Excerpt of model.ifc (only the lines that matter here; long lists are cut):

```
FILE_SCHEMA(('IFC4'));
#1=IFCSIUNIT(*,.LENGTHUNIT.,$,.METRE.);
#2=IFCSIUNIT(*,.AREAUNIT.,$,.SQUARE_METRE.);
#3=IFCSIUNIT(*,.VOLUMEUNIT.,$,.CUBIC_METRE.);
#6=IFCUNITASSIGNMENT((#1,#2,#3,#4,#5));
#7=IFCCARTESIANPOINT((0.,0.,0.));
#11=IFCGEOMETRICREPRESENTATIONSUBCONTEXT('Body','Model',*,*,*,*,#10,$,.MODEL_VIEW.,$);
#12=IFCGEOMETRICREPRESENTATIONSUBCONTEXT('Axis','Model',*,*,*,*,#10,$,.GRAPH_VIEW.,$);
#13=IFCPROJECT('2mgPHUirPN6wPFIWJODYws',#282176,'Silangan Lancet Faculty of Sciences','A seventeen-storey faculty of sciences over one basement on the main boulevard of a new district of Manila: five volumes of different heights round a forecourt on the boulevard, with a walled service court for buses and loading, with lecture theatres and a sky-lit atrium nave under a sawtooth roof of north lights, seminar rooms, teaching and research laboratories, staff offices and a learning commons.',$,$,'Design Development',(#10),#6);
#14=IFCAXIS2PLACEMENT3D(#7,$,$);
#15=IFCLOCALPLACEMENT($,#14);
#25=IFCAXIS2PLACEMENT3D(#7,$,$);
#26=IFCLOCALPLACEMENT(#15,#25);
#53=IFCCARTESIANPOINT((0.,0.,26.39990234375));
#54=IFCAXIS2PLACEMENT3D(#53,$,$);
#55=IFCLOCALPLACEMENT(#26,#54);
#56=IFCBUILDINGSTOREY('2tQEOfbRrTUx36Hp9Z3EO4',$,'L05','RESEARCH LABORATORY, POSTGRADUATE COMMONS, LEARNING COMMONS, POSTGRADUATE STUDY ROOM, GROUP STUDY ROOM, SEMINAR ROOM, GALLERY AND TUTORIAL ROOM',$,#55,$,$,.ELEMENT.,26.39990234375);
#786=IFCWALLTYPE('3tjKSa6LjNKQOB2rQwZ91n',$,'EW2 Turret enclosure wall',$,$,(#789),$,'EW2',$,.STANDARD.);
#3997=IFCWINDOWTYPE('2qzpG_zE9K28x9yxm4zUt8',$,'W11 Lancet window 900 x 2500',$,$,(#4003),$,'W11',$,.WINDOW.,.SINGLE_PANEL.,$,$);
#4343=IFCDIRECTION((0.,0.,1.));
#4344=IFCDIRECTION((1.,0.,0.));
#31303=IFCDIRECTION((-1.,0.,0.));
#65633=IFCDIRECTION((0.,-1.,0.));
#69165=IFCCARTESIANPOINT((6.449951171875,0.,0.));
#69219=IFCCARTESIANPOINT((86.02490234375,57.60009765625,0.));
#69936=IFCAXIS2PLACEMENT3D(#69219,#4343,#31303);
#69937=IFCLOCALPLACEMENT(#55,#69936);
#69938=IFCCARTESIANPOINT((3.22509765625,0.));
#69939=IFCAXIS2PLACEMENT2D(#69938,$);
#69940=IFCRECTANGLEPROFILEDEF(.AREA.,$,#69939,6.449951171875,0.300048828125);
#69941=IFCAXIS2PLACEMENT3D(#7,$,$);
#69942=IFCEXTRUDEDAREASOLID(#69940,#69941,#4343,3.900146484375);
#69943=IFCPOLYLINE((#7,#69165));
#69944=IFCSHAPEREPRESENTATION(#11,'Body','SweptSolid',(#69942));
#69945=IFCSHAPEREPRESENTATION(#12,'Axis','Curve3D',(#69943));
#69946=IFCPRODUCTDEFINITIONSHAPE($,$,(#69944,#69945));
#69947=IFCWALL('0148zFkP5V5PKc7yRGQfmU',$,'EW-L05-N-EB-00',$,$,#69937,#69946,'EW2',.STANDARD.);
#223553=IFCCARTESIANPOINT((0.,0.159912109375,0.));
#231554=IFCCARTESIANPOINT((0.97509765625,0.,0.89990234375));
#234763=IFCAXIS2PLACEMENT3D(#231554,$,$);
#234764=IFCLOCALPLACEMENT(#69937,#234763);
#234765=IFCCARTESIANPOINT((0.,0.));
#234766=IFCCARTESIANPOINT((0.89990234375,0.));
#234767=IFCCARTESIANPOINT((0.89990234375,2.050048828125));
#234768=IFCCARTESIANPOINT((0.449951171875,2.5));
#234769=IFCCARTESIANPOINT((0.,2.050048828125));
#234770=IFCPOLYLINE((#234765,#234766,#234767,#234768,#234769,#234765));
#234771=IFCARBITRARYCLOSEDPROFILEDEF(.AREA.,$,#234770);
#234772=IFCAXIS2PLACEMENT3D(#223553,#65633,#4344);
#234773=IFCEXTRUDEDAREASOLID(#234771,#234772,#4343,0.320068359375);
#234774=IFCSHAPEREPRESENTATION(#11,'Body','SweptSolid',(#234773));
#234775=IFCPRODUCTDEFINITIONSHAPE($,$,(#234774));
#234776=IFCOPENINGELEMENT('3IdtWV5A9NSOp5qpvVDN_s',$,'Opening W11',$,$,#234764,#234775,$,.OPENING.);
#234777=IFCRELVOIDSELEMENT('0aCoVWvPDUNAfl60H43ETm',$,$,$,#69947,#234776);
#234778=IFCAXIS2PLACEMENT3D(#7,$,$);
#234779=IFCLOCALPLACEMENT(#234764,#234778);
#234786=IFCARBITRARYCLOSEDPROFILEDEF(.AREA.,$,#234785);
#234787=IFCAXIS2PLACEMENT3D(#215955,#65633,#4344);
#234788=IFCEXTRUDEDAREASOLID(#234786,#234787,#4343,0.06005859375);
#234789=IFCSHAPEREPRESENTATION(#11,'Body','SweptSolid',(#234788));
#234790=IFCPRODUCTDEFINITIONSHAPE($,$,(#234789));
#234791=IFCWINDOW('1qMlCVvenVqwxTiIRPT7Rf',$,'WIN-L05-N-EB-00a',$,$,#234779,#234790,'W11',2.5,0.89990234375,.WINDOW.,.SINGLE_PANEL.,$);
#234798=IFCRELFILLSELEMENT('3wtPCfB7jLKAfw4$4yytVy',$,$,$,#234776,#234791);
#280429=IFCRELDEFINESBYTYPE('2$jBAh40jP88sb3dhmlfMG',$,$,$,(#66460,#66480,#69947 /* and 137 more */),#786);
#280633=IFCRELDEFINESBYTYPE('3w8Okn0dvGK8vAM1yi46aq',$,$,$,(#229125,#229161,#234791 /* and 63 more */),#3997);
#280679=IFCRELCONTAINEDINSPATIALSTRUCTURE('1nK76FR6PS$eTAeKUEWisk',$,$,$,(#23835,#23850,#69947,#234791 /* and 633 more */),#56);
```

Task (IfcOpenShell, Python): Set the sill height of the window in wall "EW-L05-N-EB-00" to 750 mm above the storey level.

```python
import numpy as np
import ifcopenshell
import ifcopenshell.api.geometry
import ifcopenshell.geom
import ifcopenshell.util.element
import ifcopenshell.util.placement
import ifcopenshell.util.shape
import ifcopenshell.util.unit

model = ifcopenshell.open("model.ifc")
unit_scale = ifcopenshell.util.unit.calculate_unit_scale(model)

window = model.by_id(234791)
opening = window.FillsVoids[0].RelatingOpeningElement
storey = ifcopenshell.util.element.get_container(window, ifc_class="IfcBuildingStorey")
level = ifcopenshell.util.placement.get_local_placement(storey.ObjectPlacement)[2, 3]

# The opening's origin need not be at the sill, so measure its lowest point.
shape = ifcopenshell.geom.create_shape(ifcopenshell.geom.settings(), opening)
bottom = ifcopenshell.util.shape.get_shape_bottom_elevation(shape, shape.geometry) / unit_scale
dz = level + 0.75 / unit_scale - bottom

shift = np.array([0.0, 0.0, dz])
# The window is placed relative to its opening, so it follows when the opening moves.
matrix = ifcopenshell.util.placement.get_local_placement(opening.ObjectPlacement)
matrix[:3, 3] += shift
ifcopenshell.api.geometry.edit_object_placement(
    model, product=opening, matrix=matrix, is_si=False, should_transform_children=True
)

print(f"moved by {dz * unit_scale:+.3f} m")

model.write("model_edited.ifc")
```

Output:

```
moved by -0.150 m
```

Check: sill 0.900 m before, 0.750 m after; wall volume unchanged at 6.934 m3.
